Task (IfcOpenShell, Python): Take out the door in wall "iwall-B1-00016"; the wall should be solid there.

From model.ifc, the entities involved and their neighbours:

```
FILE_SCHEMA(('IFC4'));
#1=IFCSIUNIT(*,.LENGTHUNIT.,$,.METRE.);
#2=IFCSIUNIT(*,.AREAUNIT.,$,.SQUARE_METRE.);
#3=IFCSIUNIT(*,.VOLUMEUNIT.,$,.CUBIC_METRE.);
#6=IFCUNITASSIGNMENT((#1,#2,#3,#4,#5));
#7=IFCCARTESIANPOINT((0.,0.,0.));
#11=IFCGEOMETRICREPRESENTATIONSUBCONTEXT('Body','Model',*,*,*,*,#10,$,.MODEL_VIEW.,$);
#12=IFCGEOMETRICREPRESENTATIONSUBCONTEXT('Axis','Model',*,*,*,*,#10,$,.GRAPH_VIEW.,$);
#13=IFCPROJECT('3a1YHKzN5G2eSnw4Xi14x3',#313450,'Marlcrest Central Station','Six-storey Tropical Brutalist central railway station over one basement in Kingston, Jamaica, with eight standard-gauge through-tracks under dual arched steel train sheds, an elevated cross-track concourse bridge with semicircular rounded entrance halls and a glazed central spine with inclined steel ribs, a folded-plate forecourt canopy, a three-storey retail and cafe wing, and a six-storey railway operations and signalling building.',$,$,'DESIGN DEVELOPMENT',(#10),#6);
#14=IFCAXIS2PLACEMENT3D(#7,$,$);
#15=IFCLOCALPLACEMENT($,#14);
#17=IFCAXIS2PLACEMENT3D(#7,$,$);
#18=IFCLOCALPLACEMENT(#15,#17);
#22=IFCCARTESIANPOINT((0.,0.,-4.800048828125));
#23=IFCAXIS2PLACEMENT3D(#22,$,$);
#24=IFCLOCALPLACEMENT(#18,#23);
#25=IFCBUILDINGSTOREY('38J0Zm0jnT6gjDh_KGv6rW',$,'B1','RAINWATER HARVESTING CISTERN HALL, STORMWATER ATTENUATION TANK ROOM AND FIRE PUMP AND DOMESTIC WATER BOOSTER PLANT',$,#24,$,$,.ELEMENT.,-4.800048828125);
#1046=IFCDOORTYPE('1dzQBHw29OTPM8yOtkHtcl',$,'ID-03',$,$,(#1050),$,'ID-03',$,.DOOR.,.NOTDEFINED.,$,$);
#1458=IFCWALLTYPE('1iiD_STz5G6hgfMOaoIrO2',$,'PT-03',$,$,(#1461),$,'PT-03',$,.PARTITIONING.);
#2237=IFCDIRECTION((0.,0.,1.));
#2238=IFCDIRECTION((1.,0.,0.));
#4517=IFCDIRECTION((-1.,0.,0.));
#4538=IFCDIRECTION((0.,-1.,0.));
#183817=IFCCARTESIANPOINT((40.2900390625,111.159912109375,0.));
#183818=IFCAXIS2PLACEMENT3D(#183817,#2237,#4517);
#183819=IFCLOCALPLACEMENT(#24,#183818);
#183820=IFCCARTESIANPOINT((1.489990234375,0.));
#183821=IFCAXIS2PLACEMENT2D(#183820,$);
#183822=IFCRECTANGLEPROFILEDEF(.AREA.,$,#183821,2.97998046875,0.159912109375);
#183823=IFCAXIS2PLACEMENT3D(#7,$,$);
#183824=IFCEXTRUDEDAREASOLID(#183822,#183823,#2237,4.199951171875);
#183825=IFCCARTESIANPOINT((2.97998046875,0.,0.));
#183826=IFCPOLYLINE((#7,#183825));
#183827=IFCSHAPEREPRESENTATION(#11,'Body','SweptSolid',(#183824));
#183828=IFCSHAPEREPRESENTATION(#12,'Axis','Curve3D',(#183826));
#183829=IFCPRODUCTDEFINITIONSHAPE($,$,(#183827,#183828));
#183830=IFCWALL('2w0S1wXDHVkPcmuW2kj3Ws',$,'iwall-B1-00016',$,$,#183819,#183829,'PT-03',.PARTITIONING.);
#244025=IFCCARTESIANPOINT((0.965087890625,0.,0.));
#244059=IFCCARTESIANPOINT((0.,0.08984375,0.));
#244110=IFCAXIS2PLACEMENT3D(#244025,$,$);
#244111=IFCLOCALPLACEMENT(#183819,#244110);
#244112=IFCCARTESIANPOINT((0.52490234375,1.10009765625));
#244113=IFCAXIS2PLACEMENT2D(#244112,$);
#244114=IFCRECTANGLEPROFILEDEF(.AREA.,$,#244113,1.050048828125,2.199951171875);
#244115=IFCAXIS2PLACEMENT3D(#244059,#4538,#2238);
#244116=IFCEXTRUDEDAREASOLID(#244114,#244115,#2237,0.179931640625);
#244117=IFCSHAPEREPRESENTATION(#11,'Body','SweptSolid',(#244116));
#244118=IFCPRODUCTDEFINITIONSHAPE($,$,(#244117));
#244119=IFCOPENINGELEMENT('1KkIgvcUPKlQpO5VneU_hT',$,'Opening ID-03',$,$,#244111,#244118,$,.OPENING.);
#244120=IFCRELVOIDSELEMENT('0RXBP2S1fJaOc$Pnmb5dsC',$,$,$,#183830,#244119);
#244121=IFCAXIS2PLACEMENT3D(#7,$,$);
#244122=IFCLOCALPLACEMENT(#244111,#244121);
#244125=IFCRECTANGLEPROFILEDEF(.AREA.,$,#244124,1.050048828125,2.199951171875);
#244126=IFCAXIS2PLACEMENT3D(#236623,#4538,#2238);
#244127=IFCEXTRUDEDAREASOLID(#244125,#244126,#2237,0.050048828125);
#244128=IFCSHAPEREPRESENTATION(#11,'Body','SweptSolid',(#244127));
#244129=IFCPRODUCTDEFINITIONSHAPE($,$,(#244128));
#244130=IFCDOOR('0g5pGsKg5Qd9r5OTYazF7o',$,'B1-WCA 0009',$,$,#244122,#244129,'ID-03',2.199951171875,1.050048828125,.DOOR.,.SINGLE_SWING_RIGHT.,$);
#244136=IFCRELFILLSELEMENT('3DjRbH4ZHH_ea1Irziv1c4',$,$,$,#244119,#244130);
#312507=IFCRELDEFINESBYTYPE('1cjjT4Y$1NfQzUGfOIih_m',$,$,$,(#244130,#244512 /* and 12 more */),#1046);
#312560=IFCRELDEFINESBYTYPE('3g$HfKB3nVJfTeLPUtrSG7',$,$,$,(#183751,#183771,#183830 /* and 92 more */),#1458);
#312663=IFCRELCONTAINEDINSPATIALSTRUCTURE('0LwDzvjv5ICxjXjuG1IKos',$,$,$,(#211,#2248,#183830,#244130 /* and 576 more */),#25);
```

```python
import ifcopenshell
import ifcopenshell.api.feature
import ifcopenshell.api.root
import ifcopenshell.geom
import ifcopenshell.util.shape

model = ifcopenshell.open("model.ifc")
settings = ifcopenshell.geom.settings()


def volume(element):
    """Net volume in cubic metres, openings subtracted."""
    shape = ifcopenshell.geom.create_shape(settings, element)
    return ifcopenshell.util.shape.get_volume(shape.geometry)


door = model.by_guid("0g5pGsKg5Qd9r5OTYazF7o")
opening = door.FillsVoids[0].RelatingOpeningElement
wall = opening.VoidsElements[0].RelatingBuildingElement
before = volume(wall)

ifcopenshell.api.root.remove_product(model, product=door)
ifcopenshell.api.feature.remove_feature(model, feature=opening)

after = volume(wall)

print(f"wall volume {before:.3f} -> {after:.3f} m3")

model.write("model_v2.ifc")
```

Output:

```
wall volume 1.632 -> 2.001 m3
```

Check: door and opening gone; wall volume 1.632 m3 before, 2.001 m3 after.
